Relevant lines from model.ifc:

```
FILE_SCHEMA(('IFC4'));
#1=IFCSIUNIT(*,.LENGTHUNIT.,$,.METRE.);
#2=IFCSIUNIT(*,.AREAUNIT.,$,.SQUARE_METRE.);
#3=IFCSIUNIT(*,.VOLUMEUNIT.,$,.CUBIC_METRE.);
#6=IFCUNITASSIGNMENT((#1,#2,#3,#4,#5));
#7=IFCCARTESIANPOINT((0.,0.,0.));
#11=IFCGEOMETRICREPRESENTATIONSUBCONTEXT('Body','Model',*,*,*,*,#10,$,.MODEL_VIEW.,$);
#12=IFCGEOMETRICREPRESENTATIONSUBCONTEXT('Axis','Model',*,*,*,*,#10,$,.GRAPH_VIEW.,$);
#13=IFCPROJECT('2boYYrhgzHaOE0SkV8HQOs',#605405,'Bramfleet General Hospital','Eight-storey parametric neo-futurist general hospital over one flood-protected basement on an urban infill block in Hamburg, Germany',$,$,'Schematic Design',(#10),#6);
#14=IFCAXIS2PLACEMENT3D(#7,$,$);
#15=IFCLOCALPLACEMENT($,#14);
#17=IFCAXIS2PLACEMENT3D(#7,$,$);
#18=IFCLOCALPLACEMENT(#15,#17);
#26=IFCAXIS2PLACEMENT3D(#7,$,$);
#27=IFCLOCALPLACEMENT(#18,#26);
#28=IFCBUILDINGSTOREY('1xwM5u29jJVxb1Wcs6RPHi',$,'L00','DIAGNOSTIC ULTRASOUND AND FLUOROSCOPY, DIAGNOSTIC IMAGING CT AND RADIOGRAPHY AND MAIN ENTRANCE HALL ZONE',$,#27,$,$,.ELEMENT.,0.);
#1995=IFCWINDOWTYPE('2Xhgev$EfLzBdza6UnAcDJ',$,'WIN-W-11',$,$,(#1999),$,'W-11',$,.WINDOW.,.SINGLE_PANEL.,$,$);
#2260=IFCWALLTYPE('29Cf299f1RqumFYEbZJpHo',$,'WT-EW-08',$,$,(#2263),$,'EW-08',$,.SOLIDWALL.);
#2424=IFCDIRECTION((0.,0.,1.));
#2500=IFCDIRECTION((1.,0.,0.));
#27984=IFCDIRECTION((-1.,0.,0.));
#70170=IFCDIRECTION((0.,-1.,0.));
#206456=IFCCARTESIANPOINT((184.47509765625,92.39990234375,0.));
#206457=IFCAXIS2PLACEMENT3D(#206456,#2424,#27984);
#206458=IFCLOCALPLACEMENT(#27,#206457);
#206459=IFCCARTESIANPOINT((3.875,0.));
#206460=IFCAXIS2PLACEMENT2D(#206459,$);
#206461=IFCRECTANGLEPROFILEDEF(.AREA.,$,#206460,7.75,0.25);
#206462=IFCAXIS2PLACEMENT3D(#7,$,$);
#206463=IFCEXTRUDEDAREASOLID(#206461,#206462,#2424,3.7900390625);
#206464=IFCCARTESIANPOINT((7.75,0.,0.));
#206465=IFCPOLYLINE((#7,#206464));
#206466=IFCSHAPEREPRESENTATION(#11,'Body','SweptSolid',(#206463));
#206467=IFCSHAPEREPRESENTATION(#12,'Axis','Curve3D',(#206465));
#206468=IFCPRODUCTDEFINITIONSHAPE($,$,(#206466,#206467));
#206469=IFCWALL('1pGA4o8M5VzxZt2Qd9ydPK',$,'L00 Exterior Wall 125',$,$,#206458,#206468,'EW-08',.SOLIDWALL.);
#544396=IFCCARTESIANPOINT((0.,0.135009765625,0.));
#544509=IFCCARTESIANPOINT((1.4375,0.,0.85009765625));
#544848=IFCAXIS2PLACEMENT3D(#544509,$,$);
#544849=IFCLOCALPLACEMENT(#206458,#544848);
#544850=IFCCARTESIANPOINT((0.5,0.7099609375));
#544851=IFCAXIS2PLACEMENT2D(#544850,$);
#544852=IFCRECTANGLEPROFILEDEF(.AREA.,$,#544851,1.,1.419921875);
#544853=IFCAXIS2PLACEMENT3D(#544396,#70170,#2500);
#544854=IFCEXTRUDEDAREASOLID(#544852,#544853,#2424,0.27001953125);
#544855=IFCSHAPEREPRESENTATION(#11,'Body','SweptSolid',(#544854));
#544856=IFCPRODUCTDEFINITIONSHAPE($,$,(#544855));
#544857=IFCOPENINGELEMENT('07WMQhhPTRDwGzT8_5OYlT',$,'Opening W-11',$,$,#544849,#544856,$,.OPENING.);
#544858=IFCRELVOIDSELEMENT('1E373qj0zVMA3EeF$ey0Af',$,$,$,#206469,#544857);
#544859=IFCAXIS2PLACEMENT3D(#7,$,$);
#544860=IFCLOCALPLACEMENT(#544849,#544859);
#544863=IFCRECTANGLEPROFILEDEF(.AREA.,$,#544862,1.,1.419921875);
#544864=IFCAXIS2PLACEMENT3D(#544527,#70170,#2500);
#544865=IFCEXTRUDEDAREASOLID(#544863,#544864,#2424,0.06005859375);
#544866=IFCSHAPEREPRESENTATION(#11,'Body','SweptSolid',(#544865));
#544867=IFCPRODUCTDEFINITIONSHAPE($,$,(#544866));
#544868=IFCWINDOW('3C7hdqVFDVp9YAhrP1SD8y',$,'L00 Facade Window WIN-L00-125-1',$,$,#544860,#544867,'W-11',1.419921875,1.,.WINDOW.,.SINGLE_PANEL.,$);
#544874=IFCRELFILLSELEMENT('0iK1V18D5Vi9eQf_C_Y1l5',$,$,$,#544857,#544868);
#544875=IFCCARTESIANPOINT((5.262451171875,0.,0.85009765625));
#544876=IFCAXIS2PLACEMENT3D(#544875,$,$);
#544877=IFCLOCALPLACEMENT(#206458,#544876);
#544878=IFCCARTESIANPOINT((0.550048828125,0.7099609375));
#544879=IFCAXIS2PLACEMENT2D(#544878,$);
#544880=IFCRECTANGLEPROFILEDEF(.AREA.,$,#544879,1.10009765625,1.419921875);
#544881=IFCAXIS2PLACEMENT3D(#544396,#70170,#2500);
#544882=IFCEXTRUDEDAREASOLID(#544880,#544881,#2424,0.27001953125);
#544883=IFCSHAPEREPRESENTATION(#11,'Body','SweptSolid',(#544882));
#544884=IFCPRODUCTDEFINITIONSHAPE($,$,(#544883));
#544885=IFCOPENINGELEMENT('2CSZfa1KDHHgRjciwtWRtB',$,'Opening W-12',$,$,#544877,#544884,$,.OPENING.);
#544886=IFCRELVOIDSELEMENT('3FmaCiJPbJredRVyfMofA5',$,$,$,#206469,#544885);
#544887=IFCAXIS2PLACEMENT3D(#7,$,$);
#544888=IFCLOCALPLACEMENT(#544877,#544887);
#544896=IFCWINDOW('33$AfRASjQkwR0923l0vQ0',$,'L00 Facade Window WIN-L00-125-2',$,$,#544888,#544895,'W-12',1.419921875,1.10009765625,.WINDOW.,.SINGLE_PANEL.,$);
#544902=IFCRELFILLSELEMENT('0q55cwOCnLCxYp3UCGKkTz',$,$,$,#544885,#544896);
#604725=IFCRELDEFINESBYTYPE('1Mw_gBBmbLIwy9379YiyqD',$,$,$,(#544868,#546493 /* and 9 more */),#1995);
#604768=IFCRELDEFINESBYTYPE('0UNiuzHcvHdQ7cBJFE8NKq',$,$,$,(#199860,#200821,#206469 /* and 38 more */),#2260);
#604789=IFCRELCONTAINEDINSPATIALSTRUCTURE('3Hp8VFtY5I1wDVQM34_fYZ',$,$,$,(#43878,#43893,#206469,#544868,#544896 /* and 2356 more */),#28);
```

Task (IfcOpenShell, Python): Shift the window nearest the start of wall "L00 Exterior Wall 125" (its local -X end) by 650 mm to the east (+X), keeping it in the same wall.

```python
import ifcopenshell
import ifcopenshell.api.geometry
import ifcopenshell.util.placement

model = ifcopenshell.open("model.ifc")

window = model.by_guid("3C7hdqVFDVp9YAhrP1SD8y")
opening = window.FillsVoids[0].RelatingOpeningElement
wall = opening.VoidsElements[0].RelatingBuildingElement

wall_matrix = ifcopenshell.util.placement.get_local_placement(wall.ObjectPlacement)
shift = wall_matrix[:3, 0] * -0.65
before = ifcopenshell.util.placement.get_local_placement(window.ObjectPlacement)[:3, 3].copy()

# The window is placed relative to its opening, so it follows when the opening moves.
matrix = ifcopenshell.util.placement.get_local_placement(opening.ObjectPlacement)
matrix[:3, 3] += shift
ifcopenshell.api.geometry.edit_object_placement(
    model, product=opening, matrix=matrix, is_si=False, should_transform_children=True
)

after = ifcopenshell.util.placement.get_local_placement(window.ObjectPlacement)[:3, 3]
print("window moved by", (after - before).round(3) + 0.0)

model.write("model_edited.ifc")
```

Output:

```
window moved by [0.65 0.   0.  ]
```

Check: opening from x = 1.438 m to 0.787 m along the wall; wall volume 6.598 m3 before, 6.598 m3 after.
